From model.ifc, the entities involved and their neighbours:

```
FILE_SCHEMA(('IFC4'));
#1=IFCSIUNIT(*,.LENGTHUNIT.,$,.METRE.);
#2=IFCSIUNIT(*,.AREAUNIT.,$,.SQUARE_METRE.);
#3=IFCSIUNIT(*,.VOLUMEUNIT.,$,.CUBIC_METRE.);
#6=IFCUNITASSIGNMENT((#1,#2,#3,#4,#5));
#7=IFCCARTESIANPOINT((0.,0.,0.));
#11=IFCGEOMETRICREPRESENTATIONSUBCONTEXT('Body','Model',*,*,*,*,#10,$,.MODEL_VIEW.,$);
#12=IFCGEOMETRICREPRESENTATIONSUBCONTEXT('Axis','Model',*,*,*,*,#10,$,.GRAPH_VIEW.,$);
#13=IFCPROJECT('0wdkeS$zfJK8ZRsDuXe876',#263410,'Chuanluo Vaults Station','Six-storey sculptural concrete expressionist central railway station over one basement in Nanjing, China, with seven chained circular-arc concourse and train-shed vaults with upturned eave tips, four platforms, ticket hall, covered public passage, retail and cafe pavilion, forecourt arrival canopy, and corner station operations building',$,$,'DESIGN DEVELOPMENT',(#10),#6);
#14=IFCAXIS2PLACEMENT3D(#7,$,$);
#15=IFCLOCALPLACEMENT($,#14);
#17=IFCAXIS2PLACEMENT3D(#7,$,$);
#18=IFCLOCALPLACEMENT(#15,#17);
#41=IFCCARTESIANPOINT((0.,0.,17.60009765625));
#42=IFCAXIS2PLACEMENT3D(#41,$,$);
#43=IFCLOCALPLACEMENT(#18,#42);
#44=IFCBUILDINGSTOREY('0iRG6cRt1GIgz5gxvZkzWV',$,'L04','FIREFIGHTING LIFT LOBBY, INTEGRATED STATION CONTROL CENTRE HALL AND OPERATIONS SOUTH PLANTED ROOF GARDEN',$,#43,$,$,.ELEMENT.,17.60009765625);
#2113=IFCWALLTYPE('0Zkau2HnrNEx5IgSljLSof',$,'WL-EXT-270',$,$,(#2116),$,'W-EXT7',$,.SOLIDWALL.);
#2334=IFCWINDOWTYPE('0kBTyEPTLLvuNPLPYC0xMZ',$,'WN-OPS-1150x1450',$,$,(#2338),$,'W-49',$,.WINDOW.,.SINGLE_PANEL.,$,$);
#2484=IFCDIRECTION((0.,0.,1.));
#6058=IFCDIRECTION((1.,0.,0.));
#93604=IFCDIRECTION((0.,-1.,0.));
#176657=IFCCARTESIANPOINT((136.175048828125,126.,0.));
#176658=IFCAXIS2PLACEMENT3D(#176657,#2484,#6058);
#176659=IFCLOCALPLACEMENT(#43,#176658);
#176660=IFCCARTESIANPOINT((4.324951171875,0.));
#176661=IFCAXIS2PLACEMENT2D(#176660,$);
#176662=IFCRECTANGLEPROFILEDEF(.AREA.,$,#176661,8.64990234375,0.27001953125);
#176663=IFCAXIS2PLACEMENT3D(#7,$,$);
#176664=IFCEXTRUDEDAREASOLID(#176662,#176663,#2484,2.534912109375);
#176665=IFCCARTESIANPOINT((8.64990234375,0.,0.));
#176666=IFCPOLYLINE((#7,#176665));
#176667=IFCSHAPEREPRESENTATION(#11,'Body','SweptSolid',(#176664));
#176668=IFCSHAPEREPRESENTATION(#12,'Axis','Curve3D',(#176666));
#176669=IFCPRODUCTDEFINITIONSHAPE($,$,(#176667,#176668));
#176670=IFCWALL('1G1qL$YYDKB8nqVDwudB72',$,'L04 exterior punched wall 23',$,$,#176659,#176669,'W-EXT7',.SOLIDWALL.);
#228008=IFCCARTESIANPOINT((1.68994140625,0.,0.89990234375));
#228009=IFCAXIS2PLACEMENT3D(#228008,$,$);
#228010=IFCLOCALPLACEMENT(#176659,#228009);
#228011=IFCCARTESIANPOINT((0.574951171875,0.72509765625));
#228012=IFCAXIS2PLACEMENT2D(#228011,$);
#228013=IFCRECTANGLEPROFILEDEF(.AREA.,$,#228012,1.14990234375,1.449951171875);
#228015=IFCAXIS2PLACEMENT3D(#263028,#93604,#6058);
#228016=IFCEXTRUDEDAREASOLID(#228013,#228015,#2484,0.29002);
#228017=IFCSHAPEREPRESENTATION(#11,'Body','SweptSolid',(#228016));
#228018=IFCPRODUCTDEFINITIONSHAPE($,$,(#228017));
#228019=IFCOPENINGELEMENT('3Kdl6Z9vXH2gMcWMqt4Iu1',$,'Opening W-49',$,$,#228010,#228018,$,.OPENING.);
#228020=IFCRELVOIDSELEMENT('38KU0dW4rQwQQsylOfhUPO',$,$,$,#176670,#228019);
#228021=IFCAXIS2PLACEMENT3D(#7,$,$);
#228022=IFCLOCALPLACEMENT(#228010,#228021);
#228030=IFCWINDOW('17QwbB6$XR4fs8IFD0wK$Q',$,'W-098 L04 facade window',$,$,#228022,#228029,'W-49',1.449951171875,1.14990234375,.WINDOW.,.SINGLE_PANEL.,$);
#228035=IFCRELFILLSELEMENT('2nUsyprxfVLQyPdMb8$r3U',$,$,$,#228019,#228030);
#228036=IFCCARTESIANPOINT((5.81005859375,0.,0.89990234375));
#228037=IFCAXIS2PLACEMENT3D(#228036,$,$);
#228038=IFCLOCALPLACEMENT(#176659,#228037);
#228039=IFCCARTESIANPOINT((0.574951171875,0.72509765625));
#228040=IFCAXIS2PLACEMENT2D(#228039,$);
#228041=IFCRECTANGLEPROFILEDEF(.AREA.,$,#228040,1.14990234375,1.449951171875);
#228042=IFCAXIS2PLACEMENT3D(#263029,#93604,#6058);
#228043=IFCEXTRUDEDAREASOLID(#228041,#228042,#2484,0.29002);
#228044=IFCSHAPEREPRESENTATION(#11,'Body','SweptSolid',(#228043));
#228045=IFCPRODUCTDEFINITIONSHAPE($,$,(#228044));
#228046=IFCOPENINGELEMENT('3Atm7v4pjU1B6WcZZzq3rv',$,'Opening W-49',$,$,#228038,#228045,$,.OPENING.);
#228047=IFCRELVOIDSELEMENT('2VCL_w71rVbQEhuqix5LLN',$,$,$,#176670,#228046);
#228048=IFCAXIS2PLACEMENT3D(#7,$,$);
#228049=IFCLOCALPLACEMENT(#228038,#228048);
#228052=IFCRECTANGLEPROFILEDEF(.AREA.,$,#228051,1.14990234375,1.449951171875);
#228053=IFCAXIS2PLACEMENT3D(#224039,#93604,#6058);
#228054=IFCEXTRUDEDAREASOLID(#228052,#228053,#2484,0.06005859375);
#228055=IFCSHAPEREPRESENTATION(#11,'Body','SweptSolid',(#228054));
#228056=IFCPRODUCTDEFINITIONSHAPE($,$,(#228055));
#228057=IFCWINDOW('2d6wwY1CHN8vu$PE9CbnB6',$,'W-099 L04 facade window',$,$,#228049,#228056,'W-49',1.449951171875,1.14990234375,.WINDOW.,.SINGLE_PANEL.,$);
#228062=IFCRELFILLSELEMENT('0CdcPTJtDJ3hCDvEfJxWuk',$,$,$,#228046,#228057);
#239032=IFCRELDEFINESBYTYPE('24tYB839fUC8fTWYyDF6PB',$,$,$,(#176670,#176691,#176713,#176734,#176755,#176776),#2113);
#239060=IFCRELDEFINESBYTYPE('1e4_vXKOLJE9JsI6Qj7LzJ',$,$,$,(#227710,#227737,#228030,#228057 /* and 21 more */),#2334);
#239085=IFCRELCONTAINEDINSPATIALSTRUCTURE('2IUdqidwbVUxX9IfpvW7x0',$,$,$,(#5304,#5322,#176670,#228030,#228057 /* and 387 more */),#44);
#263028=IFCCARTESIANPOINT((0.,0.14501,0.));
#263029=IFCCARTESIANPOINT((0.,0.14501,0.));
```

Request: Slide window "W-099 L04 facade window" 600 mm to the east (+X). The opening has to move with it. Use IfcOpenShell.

```python
import ifcopenshell
import ifcopenshell.api.geometry
import ifcopenshell.util.placement

model = ifcopenshell.open("model.ifc")

window = model.by_guid("2d6wwY1CHN8vu$PE9CbnB6")
opening = window.FillsVoids[0].RelatingOpeningElement
wall = opening.VoidsElements[0].RelatingBuildingElement

wall_matrix = ifcopenshell.util.placement.get_local_placement(wall.ObjectPlacement)
shift = wall_matrix[:3, 0] * 0.6
before = ifcopenshell.util.placement.get_local_placement(window.ObjectPlacement)[:3, 3].copy()

# The window is placed relative to its opening, so it follows when the opening moves.
matrix = ifcopenshell.util.placement.get_local_placement(opening.ObjectPlacement)
matrix[:3, 3] += shift
ifcopenshell.api.geometry.edit_object_placement(
    model, product=opening, matrix=matrix, is_si=False, should_transform_children=True
)

after = ifcopenshell.util.placement.get_local_placement(window.ObjectPlacement)[:3, 3]
print("window moved by", (after - before).round(3) + 0.0)

model.write("model_rev.ifc")
```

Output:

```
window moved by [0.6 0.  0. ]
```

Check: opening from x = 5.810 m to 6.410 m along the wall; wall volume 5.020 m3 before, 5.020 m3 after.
